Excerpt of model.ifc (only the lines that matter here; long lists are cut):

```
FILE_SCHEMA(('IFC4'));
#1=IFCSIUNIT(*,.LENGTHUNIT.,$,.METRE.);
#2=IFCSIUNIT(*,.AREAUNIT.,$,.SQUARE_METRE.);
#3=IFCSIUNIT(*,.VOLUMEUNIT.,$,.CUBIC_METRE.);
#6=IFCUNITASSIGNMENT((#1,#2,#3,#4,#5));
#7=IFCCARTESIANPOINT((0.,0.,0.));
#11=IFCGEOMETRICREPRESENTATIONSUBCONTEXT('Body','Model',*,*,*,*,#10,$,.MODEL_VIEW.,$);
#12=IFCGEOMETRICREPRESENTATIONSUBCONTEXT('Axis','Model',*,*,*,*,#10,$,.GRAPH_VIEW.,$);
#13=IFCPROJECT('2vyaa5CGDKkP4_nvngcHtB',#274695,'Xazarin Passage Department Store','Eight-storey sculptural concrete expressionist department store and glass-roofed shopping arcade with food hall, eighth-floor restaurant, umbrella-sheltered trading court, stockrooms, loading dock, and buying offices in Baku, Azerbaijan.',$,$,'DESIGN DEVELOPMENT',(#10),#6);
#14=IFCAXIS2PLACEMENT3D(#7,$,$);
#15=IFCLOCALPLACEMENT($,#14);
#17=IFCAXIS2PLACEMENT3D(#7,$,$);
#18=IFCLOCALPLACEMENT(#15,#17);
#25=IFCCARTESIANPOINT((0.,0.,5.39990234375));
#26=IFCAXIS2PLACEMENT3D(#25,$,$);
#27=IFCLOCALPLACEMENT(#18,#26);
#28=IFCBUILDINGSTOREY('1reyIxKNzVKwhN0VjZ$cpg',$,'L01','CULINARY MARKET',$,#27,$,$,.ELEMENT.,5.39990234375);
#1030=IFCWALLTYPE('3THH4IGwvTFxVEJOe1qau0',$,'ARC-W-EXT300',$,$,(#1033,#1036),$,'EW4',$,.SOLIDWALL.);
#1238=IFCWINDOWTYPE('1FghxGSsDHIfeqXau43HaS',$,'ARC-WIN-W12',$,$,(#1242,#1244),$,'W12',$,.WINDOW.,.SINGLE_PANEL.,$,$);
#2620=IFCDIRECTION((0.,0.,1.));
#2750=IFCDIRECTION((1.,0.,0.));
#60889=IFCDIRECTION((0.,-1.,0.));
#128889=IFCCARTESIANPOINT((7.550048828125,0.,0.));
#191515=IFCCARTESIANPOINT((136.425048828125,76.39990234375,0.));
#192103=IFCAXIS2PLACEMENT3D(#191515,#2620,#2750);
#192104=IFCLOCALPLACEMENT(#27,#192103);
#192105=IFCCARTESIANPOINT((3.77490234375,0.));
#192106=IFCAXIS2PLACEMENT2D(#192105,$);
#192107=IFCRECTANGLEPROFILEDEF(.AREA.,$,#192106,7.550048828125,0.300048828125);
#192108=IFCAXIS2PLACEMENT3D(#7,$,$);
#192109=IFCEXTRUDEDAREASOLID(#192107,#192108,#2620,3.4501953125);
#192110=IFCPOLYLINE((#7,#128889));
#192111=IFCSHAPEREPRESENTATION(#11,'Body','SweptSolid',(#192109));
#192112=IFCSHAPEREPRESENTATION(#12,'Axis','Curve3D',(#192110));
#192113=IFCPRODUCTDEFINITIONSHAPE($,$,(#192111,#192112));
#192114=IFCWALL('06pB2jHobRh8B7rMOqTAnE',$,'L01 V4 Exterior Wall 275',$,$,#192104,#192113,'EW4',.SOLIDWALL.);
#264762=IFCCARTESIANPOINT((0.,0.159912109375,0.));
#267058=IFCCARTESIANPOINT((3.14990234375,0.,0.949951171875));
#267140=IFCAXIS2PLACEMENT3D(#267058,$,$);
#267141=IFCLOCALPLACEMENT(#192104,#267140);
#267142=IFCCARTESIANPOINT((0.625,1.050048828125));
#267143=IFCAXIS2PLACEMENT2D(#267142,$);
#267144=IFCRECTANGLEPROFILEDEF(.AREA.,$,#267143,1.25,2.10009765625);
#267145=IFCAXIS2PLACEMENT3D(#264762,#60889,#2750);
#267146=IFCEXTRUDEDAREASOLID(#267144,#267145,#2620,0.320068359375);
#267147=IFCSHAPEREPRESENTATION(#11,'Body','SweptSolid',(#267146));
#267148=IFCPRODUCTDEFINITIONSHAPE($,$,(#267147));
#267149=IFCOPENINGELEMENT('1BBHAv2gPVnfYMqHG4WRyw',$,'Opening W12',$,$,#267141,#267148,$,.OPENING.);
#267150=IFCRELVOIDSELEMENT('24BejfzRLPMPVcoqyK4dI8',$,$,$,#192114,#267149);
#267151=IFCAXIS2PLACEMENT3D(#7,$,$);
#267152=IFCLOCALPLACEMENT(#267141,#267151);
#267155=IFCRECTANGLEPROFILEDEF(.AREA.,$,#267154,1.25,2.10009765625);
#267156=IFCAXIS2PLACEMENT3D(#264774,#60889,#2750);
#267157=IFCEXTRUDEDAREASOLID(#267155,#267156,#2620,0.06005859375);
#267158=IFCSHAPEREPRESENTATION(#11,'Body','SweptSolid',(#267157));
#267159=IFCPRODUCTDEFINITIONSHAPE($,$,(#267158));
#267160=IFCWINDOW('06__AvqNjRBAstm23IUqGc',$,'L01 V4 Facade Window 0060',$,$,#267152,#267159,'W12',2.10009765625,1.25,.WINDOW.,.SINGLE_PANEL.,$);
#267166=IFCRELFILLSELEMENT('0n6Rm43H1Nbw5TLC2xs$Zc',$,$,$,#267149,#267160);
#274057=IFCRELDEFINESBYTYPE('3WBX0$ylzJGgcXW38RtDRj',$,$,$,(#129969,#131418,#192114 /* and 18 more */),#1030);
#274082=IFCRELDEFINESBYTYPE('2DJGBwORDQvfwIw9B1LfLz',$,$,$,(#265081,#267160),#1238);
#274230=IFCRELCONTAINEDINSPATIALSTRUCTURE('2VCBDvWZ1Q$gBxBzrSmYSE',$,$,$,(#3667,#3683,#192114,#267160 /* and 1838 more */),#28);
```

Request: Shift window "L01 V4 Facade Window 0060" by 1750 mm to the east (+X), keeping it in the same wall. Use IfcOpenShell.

```python
import ifcopenshell
import ifcopenshell.api.geometry
import ifcopenshell.util.placement

model = ifcopenshell.open("model.ifc")

window = model.by_guid("06__AvqNjRBAstm23IUqGc")
opening = window.FillsVoids[0].RelatingOpeningElement
wall = opening.VoidsElements[0].RelatingBuildingElement

wall_matrix = ifcopenshell.util.placement.get_local_placement(wall.ObjectPlacement)
shift = wall_matrix[:3, 0] * 1.75
before = ifcopenshell.util.placement.get_local_placement(window.ObjectPlacement)[:3, 3].copy()

# The window is placed relative to its opening, so it follows when the opening moves.
matrix = ifcopenshell.util.placement.get_local_placement(opening.ObjectPlacement)
matrix[:3, 3] += shift
ifcopenshell.api.geometry.edit_object_placement(
    model, product=opening, matrix=matrix, is_si=False, should_transform_children=True
)

after = ifcopenshell.util.placement.get_local_placement(window.ObjectPlacement)[:3, 3]
print("window moved by", (after - before).round(3) + 0.0)

model.write("model-out.ifc")
```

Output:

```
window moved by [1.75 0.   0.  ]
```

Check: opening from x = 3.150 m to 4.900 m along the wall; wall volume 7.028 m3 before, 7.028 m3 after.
